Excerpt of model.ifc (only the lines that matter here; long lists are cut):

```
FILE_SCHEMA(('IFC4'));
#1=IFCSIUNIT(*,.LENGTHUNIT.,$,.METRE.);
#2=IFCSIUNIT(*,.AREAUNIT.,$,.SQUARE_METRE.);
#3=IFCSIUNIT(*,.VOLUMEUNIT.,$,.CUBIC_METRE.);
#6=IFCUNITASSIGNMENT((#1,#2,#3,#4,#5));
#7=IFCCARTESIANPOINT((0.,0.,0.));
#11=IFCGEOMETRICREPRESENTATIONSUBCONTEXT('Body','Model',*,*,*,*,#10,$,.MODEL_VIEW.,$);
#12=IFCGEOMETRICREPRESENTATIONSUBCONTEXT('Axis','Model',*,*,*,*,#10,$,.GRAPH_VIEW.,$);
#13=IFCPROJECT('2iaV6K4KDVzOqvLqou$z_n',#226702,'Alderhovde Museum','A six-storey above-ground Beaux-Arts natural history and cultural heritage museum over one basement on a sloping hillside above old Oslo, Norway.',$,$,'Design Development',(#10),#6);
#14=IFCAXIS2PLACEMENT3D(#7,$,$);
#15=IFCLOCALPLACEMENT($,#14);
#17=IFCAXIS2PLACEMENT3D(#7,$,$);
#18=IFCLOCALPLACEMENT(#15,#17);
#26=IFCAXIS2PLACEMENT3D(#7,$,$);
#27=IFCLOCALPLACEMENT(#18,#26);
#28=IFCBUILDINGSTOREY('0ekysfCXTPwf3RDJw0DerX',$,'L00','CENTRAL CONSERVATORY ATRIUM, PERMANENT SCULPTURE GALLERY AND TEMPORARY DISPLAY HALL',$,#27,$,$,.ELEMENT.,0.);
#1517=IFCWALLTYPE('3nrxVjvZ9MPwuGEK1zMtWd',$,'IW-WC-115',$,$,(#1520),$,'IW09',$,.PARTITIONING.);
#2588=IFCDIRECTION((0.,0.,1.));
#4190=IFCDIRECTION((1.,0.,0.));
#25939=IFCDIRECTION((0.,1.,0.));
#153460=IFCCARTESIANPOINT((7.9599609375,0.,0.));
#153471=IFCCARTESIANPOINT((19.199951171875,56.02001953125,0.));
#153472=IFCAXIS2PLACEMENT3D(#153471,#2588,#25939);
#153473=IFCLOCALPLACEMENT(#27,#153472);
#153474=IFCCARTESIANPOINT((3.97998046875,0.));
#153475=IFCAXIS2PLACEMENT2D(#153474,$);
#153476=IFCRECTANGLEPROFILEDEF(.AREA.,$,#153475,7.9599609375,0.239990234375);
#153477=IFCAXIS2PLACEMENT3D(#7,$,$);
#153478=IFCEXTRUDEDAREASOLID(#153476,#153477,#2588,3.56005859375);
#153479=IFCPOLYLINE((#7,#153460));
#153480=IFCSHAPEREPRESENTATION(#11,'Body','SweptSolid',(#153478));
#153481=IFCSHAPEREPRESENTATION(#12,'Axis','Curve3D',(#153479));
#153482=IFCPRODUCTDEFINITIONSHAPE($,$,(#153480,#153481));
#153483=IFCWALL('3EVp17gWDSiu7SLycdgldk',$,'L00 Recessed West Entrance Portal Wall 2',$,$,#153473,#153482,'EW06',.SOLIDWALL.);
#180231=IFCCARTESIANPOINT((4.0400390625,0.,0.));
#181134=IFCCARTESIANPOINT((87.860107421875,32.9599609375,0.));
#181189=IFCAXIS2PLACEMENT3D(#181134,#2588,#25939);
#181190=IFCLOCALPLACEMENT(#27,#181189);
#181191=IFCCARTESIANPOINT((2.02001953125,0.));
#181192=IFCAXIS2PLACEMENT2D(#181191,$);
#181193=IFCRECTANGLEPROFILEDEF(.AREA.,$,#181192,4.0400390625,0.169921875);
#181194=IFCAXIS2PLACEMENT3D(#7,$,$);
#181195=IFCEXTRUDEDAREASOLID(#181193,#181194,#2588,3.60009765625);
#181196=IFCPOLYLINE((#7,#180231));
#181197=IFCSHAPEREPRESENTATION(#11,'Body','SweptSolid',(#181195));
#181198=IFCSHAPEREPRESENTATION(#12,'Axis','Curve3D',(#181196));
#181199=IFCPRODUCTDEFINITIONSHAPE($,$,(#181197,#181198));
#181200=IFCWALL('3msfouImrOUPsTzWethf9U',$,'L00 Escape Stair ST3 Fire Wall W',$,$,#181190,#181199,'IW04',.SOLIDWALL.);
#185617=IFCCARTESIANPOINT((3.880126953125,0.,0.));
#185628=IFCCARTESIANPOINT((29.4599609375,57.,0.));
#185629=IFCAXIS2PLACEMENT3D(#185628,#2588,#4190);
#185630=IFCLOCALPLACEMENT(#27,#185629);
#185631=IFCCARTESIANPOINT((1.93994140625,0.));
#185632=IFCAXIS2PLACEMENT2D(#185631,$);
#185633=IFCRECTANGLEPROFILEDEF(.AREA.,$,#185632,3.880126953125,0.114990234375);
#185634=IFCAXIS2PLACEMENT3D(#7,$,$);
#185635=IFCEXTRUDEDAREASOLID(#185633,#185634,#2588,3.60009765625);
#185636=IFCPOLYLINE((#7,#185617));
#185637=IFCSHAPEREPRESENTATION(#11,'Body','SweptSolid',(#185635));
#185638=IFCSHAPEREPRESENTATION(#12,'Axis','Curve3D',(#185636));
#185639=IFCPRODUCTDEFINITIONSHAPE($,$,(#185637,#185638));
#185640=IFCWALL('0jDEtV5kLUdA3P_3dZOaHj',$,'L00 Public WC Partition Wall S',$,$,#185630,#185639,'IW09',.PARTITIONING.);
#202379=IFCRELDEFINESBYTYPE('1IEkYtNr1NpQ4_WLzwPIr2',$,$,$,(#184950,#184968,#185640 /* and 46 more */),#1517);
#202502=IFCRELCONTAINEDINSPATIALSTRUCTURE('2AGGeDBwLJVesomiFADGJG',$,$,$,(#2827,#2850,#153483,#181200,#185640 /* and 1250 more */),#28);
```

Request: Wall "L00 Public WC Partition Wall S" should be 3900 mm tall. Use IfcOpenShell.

```python
import ifcopenshell
import ifcopenshell.geom
import ifcopenshell.util.representation
import ifcopenshell.util.shape

model = ifcopenshell.open("model.ifc")
settings = ifcopenshell.geom.settings()


def volume(element):
    """Net volume in cubic metres, openings subtracted."""
    shape = ifcopenshell.geom.create_shape(settings, element)
    return ifcopenshell.util.shape.get_volume(shape.geometry)


wall = model.by_guid("0jDEtV5kLUdA3P_3dZOaHj")
before = volume(wall)

body = ifcopenshell.util.representation.get_representation(wall, "Model", "Body")
solid = body.Items[0]
old_height = solid.Depth
solid.Depth = 3.9
after = volume(wall)

print(f"height {old_height:g} -> {solid.Depth:g}, volume {before:.3f} -> {after:.3f} m3")

model.write("model_edited.ifc")
```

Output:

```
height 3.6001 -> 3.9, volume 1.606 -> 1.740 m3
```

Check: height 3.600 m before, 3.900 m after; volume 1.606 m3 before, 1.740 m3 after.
